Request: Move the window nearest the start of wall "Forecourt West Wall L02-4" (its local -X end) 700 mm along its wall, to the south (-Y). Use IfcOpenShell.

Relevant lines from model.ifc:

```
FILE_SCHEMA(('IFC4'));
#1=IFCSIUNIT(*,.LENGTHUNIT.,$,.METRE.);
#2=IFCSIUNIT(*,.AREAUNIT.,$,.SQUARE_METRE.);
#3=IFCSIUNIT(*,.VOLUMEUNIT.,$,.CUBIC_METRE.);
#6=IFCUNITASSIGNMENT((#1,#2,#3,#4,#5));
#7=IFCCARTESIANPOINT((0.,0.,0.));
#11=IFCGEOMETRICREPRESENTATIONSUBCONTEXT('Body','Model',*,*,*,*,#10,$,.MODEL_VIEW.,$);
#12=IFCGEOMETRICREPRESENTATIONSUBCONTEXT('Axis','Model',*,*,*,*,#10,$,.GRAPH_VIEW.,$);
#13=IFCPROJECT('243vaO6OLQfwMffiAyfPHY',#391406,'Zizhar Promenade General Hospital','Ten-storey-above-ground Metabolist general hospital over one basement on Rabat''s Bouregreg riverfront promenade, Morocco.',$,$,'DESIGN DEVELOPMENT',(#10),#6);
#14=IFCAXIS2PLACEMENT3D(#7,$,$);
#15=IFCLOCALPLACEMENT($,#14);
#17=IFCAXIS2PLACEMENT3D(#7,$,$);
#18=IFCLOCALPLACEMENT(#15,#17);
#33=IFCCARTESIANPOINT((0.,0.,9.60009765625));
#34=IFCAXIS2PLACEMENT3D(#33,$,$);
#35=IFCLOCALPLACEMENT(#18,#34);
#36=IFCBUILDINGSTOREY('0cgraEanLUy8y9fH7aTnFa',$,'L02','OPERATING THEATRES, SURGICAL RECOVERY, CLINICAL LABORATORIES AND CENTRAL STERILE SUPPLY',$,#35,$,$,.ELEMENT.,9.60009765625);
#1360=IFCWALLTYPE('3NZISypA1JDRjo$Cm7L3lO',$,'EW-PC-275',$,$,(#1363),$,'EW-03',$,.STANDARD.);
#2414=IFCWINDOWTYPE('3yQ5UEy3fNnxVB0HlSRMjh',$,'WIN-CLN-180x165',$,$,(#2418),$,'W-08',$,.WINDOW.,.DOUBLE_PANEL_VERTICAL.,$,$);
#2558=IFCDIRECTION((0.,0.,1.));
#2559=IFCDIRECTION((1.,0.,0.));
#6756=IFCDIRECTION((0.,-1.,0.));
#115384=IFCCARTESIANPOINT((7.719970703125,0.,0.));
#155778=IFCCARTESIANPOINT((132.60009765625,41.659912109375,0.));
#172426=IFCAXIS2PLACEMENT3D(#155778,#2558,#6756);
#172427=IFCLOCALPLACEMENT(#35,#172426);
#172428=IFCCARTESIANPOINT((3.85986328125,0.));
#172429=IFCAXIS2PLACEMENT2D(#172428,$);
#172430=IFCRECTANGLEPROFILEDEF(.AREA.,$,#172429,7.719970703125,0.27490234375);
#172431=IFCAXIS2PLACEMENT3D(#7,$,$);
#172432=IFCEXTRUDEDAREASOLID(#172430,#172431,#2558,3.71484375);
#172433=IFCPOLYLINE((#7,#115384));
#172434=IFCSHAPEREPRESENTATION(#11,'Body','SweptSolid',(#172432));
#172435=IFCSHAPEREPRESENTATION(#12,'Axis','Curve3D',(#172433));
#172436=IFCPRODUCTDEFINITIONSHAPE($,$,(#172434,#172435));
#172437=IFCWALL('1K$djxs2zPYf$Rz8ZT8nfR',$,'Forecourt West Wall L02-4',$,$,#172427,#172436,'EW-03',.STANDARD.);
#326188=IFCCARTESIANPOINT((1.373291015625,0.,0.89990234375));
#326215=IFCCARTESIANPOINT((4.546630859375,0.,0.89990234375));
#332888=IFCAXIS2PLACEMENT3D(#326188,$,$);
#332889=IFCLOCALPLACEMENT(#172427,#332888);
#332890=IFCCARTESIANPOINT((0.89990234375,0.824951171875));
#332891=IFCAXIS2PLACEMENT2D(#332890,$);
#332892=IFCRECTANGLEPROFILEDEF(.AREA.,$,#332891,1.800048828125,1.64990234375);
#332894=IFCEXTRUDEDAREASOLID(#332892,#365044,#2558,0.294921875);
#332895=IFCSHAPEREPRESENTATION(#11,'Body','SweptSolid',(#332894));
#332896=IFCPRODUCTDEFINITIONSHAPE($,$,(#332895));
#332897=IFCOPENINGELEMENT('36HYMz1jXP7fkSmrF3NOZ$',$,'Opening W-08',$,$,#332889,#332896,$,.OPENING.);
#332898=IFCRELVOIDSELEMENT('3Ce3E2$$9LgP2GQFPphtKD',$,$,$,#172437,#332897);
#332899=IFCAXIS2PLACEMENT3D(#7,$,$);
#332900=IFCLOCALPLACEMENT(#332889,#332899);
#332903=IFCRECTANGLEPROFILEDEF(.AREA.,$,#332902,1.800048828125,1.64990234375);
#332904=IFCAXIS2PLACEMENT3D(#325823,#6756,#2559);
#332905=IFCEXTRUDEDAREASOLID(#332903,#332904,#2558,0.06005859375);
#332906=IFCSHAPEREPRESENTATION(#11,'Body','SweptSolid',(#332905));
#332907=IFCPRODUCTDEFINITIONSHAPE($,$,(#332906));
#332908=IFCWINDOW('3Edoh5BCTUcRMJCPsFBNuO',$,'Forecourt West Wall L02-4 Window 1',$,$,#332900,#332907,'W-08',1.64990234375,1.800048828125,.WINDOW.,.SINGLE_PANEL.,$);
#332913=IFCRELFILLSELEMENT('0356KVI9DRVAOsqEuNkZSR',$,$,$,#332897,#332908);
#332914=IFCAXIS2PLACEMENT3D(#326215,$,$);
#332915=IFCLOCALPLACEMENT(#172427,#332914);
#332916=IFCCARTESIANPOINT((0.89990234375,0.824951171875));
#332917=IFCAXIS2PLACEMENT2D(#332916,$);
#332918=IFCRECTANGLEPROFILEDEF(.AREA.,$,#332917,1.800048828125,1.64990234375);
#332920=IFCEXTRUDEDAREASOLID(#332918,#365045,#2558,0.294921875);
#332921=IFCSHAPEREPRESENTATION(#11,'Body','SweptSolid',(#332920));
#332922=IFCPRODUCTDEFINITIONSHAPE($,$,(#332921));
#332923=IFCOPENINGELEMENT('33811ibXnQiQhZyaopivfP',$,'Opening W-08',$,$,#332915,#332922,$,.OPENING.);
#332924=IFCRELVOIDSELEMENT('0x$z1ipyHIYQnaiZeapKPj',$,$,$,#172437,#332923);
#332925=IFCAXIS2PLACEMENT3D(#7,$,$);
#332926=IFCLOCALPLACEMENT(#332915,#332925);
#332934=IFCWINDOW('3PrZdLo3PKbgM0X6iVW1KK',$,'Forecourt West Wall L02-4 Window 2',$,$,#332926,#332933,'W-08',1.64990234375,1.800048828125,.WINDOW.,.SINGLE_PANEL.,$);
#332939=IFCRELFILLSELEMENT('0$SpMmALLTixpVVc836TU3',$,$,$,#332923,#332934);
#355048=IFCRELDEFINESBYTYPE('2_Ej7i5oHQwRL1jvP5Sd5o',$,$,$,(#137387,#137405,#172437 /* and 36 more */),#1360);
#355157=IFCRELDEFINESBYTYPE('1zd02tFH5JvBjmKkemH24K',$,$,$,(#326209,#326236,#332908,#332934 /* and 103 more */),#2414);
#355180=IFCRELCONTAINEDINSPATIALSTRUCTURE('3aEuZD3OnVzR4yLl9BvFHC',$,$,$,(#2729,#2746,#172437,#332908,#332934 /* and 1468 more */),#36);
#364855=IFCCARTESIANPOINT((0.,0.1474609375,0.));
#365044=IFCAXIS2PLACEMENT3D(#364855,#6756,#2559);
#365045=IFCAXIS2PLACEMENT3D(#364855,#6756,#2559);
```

```python
import ifcopenshell
import ifcopenshell.api.geometry
import ifcopenshell.util.placement
import ifcopenshell.util.unit

model = ifcopenshell.open("model.ifc")
unit_scale = ifcopenshell.util.unit.calculate_unit_scale(model)

window = model.by_guid("3Edoh5BCTUcRMJCPsFBNuO")
opening = window.FillsVoids[0].RelatingOpeningElement
wall = opening.VoidsElements[0].RelatingBuildingElement

wall_matrix = ifcopenshell.util.placement.get_local_placement(wall.ObjectPlacement)
shift = wall_matrix[:3, 0] * 0.7 / unit_scale
before = ifcopenshell.util.placement.get_local_placement(window.ObjectPlacement)[:3, 3].copy()

# The window is placed relative to its opening, so it follows when the opening moves.
matrix = ifcopenshell.util.placement.get_local_placement(opening.ObjectPlacement)
matrix[:3, 3] += shift
ifcopenshell.api.geometry.edit_object_placement(
    model, product=opening, matrix=matrix, is_si=False, should_transform_children=True
)

after = ifcopenshell.util.placement.get_local_placement(window.ObjectPlacement)[:3, 3]
print("window moved by", (after - before).round(3) + 0.0)

model.write("model_rev.ifc")
```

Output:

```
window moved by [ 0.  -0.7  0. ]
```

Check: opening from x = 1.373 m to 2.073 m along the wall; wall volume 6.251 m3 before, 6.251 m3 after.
